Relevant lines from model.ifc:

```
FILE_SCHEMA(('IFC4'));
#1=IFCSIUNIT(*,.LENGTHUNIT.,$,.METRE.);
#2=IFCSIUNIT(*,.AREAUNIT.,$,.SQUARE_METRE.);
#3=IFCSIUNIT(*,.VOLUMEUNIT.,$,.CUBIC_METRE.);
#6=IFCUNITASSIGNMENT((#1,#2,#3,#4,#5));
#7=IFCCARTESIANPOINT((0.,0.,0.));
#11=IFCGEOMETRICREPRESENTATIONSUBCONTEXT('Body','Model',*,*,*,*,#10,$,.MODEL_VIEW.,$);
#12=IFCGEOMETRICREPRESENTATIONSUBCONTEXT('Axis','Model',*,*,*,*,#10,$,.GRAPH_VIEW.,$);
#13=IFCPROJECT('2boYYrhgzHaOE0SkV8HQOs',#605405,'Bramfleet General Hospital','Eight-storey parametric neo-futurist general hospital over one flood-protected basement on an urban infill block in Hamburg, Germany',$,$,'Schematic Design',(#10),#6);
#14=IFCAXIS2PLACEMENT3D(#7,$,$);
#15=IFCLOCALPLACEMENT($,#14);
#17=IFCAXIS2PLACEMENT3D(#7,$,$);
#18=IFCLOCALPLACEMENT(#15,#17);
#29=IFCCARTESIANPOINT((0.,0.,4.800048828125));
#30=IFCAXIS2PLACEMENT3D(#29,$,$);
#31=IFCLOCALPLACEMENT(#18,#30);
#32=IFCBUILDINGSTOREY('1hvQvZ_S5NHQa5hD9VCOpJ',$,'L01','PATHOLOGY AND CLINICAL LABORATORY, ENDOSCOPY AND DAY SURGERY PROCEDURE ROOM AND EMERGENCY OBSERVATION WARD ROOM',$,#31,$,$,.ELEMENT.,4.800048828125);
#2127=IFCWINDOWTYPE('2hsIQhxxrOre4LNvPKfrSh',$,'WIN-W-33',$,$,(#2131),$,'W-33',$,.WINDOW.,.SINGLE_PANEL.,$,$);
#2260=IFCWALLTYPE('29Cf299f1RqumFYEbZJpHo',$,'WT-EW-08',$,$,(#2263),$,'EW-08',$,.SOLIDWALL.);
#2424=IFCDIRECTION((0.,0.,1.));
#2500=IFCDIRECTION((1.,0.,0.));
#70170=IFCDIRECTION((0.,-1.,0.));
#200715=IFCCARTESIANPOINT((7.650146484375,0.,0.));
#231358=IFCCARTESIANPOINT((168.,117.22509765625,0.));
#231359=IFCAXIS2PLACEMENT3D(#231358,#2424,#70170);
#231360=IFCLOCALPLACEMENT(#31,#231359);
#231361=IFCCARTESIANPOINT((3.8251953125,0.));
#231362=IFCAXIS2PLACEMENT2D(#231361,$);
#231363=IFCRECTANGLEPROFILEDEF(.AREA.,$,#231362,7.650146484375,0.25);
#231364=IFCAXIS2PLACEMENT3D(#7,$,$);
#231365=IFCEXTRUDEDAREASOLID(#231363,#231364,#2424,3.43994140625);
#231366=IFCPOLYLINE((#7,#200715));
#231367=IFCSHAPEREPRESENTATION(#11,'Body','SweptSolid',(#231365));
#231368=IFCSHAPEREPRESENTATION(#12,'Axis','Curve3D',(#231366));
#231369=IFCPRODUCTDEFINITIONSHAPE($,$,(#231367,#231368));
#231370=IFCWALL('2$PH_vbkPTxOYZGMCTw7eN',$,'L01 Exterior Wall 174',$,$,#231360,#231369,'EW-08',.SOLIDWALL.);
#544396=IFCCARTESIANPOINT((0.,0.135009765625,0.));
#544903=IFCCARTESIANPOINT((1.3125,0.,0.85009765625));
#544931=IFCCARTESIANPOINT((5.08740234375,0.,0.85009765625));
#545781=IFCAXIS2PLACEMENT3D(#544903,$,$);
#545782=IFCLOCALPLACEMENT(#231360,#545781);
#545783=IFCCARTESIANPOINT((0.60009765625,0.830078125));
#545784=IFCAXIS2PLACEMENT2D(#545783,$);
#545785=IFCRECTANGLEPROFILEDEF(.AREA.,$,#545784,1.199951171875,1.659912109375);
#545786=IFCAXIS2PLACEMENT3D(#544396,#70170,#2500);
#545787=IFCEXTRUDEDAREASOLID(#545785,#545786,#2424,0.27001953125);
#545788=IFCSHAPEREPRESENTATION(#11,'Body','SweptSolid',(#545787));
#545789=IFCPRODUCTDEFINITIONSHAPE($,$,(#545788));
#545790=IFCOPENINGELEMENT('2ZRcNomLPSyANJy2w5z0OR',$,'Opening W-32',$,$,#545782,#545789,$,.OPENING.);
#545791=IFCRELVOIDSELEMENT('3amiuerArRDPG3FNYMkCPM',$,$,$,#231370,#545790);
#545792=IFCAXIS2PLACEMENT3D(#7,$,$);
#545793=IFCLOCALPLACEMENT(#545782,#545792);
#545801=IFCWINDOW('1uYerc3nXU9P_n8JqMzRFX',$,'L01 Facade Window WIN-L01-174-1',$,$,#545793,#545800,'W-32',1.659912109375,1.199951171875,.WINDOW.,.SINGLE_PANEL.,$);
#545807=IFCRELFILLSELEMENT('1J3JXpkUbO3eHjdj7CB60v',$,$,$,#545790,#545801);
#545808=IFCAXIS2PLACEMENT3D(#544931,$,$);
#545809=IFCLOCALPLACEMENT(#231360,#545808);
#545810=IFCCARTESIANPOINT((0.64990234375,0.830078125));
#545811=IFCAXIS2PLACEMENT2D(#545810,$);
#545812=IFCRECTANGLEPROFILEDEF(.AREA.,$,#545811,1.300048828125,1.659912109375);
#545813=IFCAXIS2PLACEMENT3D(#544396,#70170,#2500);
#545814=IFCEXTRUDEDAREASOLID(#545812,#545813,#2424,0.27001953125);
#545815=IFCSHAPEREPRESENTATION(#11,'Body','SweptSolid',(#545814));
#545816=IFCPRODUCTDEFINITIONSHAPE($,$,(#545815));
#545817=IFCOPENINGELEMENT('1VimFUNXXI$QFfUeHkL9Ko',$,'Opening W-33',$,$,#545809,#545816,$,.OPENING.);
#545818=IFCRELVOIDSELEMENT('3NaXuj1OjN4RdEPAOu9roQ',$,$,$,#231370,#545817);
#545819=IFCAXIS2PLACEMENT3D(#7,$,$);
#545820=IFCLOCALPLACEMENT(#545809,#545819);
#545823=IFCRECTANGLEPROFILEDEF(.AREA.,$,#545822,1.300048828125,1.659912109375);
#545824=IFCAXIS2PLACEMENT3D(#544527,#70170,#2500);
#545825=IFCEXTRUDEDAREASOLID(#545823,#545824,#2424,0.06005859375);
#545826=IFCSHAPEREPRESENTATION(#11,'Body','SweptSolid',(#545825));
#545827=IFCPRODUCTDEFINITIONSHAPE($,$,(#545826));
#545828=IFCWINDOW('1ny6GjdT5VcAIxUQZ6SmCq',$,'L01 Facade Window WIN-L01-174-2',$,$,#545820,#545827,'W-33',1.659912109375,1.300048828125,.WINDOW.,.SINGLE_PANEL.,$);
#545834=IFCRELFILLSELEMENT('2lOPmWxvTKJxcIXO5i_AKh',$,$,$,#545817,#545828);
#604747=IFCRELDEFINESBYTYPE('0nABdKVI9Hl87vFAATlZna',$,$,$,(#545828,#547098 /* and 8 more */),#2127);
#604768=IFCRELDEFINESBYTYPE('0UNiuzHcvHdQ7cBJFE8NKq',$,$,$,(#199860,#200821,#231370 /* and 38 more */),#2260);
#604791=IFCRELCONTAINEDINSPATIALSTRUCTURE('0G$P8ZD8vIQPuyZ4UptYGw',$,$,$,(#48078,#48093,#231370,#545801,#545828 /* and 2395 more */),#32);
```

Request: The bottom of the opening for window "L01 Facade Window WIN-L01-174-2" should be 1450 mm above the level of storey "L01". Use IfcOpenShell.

```python
import numpy as np
import ifcopenshell
import ifcopenshell.api.geometry
import ifcopenshell.geom
import ifcopenshell.util.element
import ifcopenshell.util.placement
import ifcopenshell.util.shape
import ifcopenshell.util.unit

model = ifcopenshell.open("model.ifc")
unit_scale = ifcopenshell.util.unit.calculate_unit_scale(model)

window = model.by_guid("1ny6GjdT5VcAIxUQZ6SmCq")
opening = window.FillsVoids[0].RelatingOpeningElement
storey = ifcopenshell.util.element.get_container(window, ifc_class="IfcBuildingStorey")
level = ifcopenshell.util.placement.get_local_placement(storey.ObjectPlacement)[2, 3]

# The opening's origin need not be at the sill, so measure its lowest point.
shape = ifcopenshell.geom.create_shape(ifcopenshell.geom.settings(), opening)
bottom = ifcopenshell.util.shape.get_shape_bottom_elevation(shape, shape.geometry) / unit_scale
dz = level + 1.45 / unit_scale - bottom

shift = np.array([0.0, 0.0, dz])
# The window is placed relative to its opening, so it follows when the opening moves.
matrix = ifcopenshell.util.placement.get_local_placement(opening.ObjectPlacement)
matrix[:3, 3] += shift
ifcopenshell.api.geometry.edit_object_placement(
    model, product=opening, matrix=matrix, is_si=False, should_transform_children=True
)

print(f"moved by {dz * unit_scale:+.3f} m")

model.write("model_v2.ifc")
```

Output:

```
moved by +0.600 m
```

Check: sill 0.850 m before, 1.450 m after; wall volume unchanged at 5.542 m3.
